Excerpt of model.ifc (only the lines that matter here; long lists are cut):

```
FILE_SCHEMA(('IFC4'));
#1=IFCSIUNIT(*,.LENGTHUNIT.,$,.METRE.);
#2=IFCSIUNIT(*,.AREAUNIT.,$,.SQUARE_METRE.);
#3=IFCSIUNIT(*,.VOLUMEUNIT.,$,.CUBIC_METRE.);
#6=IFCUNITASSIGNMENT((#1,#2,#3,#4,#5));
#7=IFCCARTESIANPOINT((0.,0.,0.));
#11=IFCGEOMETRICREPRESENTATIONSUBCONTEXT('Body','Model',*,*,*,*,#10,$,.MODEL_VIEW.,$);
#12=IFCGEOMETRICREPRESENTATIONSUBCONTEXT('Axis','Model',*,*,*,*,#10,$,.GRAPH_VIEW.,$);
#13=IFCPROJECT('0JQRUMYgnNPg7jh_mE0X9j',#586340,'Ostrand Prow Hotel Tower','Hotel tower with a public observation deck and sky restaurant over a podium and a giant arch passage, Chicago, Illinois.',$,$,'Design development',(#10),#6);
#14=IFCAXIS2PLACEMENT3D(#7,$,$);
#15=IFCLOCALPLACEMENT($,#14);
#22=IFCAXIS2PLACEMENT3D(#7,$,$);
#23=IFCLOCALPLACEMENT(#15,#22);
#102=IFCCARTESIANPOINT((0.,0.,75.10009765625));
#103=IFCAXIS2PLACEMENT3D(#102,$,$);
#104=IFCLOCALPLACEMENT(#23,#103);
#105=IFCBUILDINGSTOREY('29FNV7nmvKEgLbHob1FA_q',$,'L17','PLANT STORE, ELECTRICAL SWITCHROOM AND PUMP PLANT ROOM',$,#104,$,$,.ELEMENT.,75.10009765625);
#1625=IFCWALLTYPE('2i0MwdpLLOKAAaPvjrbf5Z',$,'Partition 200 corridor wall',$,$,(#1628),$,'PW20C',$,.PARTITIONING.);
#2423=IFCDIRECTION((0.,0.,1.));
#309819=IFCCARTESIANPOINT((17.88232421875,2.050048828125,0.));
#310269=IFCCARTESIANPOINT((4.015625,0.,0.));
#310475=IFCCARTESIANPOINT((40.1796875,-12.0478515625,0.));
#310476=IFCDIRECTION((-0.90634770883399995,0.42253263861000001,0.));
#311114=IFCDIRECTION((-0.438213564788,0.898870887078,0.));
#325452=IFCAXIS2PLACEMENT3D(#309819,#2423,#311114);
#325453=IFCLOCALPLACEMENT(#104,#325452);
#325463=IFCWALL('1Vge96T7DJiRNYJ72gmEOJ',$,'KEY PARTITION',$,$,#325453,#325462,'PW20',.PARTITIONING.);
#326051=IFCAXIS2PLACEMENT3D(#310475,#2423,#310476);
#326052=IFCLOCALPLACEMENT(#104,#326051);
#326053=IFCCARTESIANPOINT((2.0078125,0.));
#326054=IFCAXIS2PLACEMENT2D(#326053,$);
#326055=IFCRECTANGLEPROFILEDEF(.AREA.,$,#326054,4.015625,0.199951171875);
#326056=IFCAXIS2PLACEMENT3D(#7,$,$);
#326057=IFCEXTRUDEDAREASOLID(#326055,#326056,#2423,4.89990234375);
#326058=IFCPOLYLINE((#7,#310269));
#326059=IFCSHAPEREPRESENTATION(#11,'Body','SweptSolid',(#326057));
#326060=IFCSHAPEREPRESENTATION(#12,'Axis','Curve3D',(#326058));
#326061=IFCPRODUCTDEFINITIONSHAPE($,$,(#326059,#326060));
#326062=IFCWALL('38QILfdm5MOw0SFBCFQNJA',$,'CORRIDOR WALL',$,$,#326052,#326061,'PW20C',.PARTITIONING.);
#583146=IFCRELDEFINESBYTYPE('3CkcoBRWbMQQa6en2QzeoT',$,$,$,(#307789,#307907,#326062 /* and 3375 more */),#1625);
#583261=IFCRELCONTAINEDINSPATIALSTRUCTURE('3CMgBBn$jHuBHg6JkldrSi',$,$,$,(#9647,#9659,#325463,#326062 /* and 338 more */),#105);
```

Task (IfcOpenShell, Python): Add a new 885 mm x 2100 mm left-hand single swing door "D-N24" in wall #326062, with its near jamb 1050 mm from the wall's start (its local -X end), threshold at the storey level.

```python
import numpy as np
import ifcopenshell
import ifcopenshell.api.feature
import ifcopenshell.api.geometry
import ifcopenshell.api.root
import ifcopenshell.api.spatial
import ifcopenshell.geom
import ifcopenshell.util.element
import ifcopenshell.util.placement
import ifcopenshell.util.representation
import ifcopenshell.util.shape
import ifcopenshell.util.unit

model = ifcopenshell.open("model.ifc")
unit_scale = ifcopenshell.util.unit.calculate_unit_scale(model)
settings = ifcopenshell.geom.settings()


def volume(element):
    """Net volume in cubic metres, openings subtracted."""
    shape = ifcopenshell.geom.create_shape(settings, element)
    return ifcopenshell.util.shape.get_volume(shape.geometry)


wall = model.by_guid("38QILfdm5MOw0SFBCFQNJA")
storey = ifcopenshell.util.element.get_container(wall, ifc_class="IfcBuildingStorey")
context = ifcopenshell.util.representation.get_context(model, "Model", "Body", "MODEL_VIEW")
before = volume(wall)

width, height, from_end, sill = 0.885, 2.1, 1.05, 0.0  # metres

# The wall runs along its own X axis, and the end named is its -X end.
wall_shape = ifcopenshell.geom.create_shape(settings, wall)
x, y, z = ifcopenshell.util.shape.get_vertices(wall_shape.geometry).T
start = x.min() + from_end
face, thickness = float(y.min()), float(y.max() - y.min())
wall_matrix = ifcopenshell.util.placement.get_local_placement(wall.ObjectPlacement)
level = ifcopenshell.util.placement.get_local_placement(storey.ObjectPlacement)[2, 3]


def in_wall(x, y):
    """Placement at x, y metres in the wall's axes, at sill height."""
    matrix = wall_matrix.copy()
    matrix[:, 3] = wall_matrix @ np.array([x / unit_scale, y / unit_scale, 0.0, 1.0])
    matrix[2, 3] = level + sill / unit_scale
    return matrix


# Opening: a box that overshoots both wall faces by 50 mm.
opening = ifcopenshell.api.root.create_entity(model, ifc_class="IfcOpeningElement", predefined_type="OPENING")
box = ifcopenshell.api.geometry.add_wall_representation(
    model, context=context, length=width, height=height, thickness=thickness + 0.1
)
ifcopenshell.api.geometry.assign_representation(model, product=opening, representation=box)
ifcopenshell.api.geometry.edit_object_placement(model, product=opening, matrix=in_wall(start, face - 0.05), is_si=False)
ifcopenshell.api.feature.add_feature(model, feature=opening, element=wall)

door = ifcopenshell.api.root.create_entity(model, ifc_class="IfcDoor", name="D-N24", predefined_type="DOOR")
door.OverallWidth, door.OverallHeight = width / unit_scale, height / unit_scale
door.OperationType = "SINGLE_SWING_LEFT"
body = ifcopenshell.api.geometry.add_door_representation(
    model,
    context=context,
    overall_width=door.OverallWidth,
    overall_height=door.OverallHeight,
    operation_type="SINGLE_SWING_LEFT",
    lining_properties={"LiningDepth": thickness / unit_scale, "ThresholdDepth": thickness / unit_scale},
)
ifcopenshell.api.geometry.assign_representation(model, product=door, representation=body)
ifcopenshell.api.spatial.assign_container(model, products=[door], relating_structure=storey)
ifcopenshell.api.feature.add_filling(model, opening=opening, element=door)

# The lining spans the wall, so the door starts at the wall face.
ifcopenshell.api.geometry.edit_object_placement(model, product=door, matrix=in_wall(start, face), is_si=False)

after = volume(wall)

print(f"wall volume {before:.3f} -> {after:.3f} m3")

model.write("model_v2.ifc")
```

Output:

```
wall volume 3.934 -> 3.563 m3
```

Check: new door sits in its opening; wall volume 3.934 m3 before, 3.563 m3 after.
